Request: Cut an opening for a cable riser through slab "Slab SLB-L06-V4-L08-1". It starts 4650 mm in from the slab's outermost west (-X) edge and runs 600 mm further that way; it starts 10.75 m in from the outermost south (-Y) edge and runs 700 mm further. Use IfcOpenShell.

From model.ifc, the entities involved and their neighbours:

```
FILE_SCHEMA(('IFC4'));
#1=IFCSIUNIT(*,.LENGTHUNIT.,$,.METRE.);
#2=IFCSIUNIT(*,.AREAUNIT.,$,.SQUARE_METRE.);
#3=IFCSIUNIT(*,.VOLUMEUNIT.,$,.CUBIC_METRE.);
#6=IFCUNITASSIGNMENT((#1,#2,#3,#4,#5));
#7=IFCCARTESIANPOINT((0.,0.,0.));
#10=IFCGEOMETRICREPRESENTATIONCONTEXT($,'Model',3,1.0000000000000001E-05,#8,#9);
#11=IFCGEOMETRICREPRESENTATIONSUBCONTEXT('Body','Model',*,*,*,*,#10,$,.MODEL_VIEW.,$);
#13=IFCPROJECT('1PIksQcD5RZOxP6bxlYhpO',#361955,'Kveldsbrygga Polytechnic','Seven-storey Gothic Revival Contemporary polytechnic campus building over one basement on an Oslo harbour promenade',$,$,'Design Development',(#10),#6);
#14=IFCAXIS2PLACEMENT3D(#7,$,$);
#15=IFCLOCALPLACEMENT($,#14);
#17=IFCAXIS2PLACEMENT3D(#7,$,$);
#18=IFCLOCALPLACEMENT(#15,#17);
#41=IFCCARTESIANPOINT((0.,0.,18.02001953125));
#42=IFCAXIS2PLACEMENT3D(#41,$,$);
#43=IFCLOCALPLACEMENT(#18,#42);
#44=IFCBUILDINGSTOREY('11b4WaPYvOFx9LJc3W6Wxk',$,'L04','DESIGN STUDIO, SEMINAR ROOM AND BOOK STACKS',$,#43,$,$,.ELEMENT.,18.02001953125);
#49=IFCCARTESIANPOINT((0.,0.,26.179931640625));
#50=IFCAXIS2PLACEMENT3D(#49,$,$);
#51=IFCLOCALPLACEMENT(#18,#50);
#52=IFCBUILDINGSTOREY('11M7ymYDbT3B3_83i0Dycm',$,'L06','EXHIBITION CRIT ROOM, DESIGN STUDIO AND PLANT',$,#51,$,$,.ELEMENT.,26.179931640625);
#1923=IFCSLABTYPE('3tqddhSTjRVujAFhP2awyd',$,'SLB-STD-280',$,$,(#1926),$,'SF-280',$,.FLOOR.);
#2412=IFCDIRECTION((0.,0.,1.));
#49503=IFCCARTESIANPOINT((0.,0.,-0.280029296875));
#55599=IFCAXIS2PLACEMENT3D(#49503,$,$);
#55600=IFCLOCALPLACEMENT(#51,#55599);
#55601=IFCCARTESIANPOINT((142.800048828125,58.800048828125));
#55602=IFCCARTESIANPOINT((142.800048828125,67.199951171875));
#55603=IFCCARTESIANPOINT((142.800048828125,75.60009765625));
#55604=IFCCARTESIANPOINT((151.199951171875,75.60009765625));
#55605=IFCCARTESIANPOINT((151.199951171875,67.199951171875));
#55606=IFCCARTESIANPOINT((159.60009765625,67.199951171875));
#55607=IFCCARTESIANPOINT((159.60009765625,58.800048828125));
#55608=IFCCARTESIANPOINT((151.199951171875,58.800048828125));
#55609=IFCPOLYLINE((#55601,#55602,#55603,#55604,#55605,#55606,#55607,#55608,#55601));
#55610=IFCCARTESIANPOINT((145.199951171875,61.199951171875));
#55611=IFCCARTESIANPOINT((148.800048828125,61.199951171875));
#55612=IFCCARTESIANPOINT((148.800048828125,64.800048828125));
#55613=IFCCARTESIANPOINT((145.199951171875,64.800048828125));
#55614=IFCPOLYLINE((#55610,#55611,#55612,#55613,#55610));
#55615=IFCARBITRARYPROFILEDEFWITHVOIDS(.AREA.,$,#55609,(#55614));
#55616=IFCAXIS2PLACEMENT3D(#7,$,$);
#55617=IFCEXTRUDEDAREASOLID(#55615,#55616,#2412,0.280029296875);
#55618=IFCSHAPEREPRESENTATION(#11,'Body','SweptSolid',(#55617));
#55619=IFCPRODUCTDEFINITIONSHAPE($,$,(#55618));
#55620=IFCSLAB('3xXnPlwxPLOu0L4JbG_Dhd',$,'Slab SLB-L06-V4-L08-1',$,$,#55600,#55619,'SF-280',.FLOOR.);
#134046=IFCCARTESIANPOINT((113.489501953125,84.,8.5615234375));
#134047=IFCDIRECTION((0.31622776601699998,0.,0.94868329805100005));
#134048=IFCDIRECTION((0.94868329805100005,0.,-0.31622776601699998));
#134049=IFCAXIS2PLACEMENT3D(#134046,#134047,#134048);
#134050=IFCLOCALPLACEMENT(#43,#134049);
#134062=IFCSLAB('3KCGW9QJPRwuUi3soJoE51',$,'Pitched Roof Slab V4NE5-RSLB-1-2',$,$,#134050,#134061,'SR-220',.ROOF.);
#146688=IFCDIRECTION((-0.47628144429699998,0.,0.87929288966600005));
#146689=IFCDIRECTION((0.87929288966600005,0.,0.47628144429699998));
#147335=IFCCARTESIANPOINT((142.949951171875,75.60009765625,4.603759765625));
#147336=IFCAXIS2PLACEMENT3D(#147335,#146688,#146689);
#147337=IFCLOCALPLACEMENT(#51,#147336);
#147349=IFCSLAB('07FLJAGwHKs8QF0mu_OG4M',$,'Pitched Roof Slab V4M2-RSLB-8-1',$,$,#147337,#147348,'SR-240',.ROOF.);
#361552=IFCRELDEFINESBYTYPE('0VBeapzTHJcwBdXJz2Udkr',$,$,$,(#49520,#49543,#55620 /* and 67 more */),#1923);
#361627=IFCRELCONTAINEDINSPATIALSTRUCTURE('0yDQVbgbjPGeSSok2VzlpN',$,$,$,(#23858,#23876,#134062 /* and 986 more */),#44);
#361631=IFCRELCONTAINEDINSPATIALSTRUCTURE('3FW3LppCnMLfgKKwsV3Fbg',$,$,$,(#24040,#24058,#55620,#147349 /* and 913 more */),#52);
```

```python
import numpy as np
import ifcopenshell
import ifcopenshell.api.feature
import ifcopenshell.api.geometry
import ifcopenshell.api.root
import ifcopenshell.geom
import ifcopenshell.util.placement
import ifcopenshell.util.representation
import ifcopenshell.util.shape
import ifcopenshell.util.unit

model = ifcopenshell.open("model.ifc")
unit_scale = ifcopenshell.util.unit.calculate_unit_scale(model)
settings = ifcopenshell.geom.settings()


def volume(element):
    """Net volume in cubic metres, openings subtracted."""
    shape = ifcopenshell.geom.create_shape(settings, element)
    return ifcopenshell.util.shape.get_volume(shape.geometry)


slab = model.by_guid("3xXnPlwxPLOu0L4JbG_Dhd")
before = volume(slab)

# Extent in the slab's own axes, in metres. The edges named are its -X and -Y sides.
slab_shape = ifcopenshell.geom.create_shape(settings, slab)
vertices = ifcopenshell.util.shape.get_vertices(slab_shape.geometry)
x_min, y_min, bottom = vertices.min(axis=0)
top = vertices[:, 2].max()

opening = ifcopenshell.api.root.create_entity(model, ifc_class="IfcOpeningElement", name="Cable riser opening", predefined_type="OPENING")
context = ifcopenshell.util.representation.get_context(model, "Model", "Body", "MODEL_VIEW")
width, depth = 0.6, 0.7
outline = [(0.0, 0.0), (width, 0.0), (width, depth), (0.0, depth), (0.0, 0.0)]
# Overshoot both faces by 50 mm so the cut is clean.
shape = ifcopenshell.api.geometry.add_slab_representation(
    model, context=context, depth=top - bottom + 0.1, polyline=outline
)
ifcopenshell.api.geometry.assign_representation(model, product=opening, representation=shape)

matrix = ifcopenshell.util.placement.get_local_placement(slab.ObjectPlacement)
matrix[:, 3] = matrix @ np.append(np.array([x_min + 4.65, y_min + 10.75, bottom - 0.05]) / unit_scale, 1.0)
ifcopenshell.api.geometry.edit_object_placement(model, product=opening, matrix=matrix, is_si=False)
ifcopenshell.api.feature.add_feature(model, feature=opening, element=slab)

after = volume(slab)

print(f"slab volume {before:.3f} -> {after:.3f} m3")

model.write("model_edited.ifc")
```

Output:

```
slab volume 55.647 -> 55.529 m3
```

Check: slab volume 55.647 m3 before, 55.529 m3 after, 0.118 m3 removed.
